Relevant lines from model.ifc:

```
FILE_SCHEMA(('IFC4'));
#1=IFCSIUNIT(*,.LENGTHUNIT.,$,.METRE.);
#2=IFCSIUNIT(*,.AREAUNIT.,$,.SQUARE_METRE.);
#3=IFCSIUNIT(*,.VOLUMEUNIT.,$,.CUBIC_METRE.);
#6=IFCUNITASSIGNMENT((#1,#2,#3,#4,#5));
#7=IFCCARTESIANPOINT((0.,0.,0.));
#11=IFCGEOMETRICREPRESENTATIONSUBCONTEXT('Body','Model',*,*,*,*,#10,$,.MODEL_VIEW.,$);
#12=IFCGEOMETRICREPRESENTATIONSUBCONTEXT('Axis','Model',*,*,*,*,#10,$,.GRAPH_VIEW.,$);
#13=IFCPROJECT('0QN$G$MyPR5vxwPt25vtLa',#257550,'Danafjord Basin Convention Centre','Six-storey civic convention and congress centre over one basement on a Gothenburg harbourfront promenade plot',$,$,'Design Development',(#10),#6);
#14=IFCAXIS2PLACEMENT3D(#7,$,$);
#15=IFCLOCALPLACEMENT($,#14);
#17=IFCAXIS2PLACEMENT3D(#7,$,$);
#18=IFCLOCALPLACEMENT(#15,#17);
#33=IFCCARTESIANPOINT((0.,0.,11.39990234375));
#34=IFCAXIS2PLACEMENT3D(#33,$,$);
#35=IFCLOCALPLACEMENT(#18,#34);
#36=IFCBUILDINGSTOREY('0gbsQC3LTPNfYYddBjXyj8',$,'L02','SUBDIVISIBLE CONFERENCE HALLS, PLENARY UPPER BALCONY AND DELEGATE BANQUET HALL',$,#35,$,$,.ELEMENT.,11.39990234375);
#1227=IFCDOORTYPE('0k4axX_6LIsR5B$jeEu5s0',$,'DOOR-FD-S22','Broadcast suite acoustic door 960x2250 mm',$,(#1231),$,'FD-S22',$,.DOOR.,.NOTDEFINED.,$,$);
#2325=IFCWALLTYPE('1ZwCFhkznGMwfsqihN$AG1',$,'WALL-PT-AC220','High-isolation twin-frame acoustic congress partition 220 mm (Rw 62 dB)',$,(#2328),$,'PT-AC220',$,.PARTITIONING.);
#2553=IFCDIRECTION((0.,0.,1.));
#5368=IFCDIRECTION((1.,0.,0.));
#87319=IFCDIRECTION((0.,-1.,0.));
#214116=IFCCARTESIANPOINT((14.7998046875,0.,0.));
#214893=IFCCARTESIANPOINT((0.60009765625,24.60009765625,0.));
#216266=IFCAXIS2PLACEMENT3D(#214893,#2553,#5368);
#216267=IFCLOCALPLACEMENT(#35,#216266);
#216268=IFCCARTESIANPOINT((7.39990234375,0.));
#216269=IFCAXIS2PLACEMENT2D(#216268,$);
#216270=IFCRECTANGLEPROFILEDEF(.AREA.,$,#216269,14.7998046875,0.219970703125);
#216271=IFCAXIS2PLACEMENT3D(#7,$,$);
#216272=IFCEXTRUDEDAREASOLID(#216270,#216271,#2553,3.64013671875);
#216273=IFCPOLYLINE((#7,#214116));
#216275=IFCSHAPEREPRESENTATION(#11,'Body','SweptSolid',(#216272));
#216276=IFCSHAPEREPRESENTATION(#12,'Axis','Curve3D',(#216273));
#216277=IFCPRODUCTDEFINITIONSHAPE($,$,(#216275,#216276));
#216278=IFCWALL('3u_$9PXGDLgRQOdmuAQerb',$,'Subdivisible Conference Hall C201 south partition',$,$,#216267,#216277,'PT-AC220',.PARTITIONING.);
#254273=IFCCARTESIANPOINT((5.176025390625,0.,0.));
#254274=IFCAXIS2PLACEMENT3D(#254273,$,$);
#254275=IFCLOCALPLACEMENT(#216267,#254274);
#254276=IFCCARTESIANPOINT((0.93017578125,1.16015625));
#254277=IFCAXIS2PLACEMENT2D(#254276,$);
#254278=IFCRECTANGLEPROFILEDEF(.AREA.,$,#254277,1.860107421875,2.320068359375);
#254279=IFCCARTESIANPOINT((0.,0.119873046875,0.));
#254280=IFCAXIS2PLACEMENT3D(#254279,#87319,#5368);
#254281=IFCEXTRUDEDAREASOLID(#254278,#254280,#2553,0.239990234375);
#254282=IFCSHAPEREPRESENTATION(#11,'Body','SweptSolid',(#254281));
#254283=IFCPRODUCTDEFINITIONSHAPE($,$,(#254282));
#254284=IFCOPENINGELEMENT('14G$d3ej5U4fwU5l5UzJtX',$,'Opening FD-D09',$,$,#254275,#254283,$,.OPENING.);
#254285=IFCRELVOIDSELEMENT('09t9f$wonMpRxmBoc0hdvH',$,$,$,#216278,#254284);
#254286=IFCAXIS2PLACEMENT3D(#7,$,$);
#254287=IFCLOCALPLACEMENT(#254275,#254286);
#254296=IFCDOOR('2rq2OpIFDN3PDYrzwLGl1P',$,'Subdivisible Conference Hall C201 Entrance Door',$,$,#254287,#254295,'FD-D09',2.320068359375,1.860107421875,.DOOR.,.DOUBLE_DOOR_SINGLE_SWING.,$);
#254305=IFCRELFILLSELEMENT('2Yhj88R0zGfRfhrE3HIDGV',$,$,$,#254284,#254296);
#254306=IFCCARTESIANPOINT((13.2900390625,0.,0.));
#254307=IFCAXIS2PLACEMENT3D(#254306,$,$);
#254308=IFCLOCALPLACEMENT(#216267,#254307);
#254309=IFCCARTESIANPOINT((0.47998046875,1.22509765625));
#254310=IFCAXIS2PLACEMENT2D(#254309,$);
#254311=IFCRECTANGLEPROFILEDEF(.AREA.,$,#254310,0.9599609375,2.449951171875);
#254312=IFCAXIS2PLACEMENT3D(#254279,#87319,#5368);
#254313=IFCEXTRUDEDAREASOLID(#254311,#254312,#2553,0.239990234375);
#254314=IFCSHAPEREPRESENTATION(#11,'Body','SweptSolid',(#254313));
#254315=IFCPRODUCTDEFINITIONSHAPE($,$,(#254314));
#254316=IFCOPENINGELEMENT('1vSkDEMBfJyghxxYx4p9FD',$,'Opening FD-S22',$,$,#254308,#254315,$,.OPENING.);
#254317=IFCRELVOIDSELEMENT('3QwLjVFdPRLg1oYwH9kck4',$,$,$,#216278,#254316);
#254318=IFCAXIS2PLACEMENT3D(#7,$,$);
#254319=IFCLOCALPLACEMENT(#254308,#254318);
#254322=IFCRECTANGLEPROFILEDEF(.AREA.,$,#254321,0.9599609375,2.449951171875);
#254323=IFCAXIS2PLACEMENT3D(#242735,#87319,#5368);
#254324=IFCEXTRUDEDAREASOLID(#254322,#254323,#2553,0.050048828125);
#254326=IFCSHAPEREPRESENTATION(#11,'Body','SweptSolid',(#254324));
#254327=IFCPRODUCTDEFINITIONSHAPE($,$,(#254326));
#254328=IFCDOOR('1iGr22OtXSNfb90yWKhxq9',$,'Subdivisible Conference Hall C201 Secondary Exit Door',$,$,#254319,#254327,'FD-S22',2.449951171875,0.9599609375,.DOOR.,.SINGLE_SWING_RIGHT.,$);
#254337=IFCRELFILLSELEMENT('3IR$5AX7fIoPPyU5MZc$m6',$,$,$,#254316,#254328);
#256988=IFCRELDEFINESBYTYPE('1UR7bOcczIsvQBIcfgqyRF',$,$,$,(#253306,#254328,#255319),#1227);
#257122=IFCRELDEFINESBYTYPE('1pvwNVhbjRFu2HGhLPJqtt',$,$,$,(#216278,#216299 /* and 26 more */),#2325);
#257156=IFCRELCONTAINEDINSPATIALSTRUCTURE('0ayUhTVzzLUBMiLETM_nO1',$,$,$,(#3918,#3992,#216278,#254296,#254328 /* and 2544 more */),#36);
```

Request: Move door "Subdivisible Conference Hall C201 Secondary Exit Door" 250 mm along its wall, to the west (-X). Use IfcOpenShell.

```python
import ifcopenshell
import ifcopenshell.api.geometry
import ifcopenshell.util.placement
import ifcopenshell.util.unit

model = ifcopenshell.open("model.ifc")
unit_scale = ifcopenshell.util.unit.calculate_unit_scale(model)

door = model.by_guid("1iGr22OtXSNfb90yWKhxq9")
opening = door.FillsVoids[0].RelatingOpeningElement
wall = opening.VoidsElements[0].RelatingBuildingElement

wall_matrix = ifcopenshell.util.placement.get_local_placement(wall.ObjectPlacement)
shift = wall_matrix[:3, 0] * -0.25 / unit_scale
before = ifcopenshell.util.placement.get_local_placement(door.ObjectPlacement)[:3, 3].copy()

# The door is placed relative to its opening, so it follows when the opening moves.
matrix = ifcopenshell.util.placement.get_local_placement(opening.ObjectPlacement)
matrix[:3, 3] += shift
ifcopenshell.api.geometry.edit_object_placement(
    model, product=opening, matrix=matrix, is_si=False, should_transform_children=True
)

after = ifcopenshell.util.placement.get_local_placement(door.ObjectPlacement)[:3, 3]
print("door moved by", (after - before).round(3) + 0.0)

model.write("model_edited.ifc")
```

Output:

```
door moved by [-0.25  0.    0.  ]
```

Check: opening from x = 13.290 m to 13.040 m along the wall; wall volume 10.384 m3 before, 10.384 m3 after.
